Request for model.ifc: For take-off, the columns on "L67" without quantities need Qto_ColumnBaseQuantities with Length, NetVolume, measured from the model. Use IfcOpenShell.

First a look at what the model holds.

```python
import ifcopenshell
import ifcopenshell.util.element
import ifcopenshell.util.unit

model = ifcopenshell.open("model.ifc")
print(model.schema)
for unit_type in ("LENGTHUNIT", "AREAUNIT", "VOLUMEUNIT"):
    print(unit_type, ifcopenshell.util.unit.calculate_unit_scale(model, unit_type))
storey = next(s for s in model.by_type("IfcBuildingStorey") if s.Name == "L67")
columns = [e for e in ifcopenshell.util.element.get_decomposition(storey) if e.is_a("IfcColumn")]
for e in sorted(columns, key=lambda e: e.id()):
    print(e.id(), e.is_a(), e.Name, list(ifcopenshell.util.element.get_psets(e, qtos_only=True)), sep=" | ")
```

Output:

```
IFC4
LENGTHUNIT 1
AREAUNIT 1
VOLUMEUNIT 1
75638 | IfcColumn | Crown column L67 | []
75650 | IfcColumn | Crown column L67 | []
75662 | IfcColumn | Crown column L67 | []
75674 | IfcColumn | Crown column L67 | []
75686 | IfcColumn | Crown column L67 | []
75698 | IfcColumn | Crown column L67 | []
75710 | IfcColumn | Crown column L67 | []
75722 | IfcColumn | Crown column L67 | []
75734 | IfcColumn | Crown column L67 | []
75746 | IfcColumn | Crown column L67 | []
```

```python
import ifcopenshell
import ifcopenshell.api.pset
import ifcopenshell.geom
import ifcopenshell.util.element
import ifcopenshell.util.shape
import ifcopenshell.util.unit

model = ifcopenshell.open("model.ifc")
unit_scale = ifcopenshell.util.unit.calculate_unit_scale(model)
volume_scale = ifcopenshell.util.unit.calculate_unit_scale(model, "VOLUMEUNIT")
settings = ifcopenshell.geom.settings()

storey = next(s for s in model.by_type("IfcBuildingStorey") if s.Name == "L67")
columns = [e for e in ifcopenshell.util.element.get_decomposition(storey) if e.is_a("IfcColumn")]

for e in sorted(columns, key=lambda e: e.id()):
    if ifcopenshell.util.element.get_psets(e, qtos_only=True, should_inherit=False):
        continue
    # Geometry comes back in metres, in the element's own axes.
    shape = ifcopenshell.geom.create_shape(settings, e)
    values = {
        "Length": ifcopenshell.util.shape.get_z(shape.geometry) / unit_scale,
        "NetVolume": ifcopenshell.util.shape.get_volume(shape.geometry) / volume_scale,
    }
    qto = ifcopenshell.api.pset.add_qto(model, product=e, name="Qto_ColumnBaseQuantities")
    ifcopenshell.api.pset.edit_qto(model, qto=qto, properties=values)
    print(e.id(), {k: round(v, 3) for k, v in values.items()})

model.write("model_rev.ifc")
```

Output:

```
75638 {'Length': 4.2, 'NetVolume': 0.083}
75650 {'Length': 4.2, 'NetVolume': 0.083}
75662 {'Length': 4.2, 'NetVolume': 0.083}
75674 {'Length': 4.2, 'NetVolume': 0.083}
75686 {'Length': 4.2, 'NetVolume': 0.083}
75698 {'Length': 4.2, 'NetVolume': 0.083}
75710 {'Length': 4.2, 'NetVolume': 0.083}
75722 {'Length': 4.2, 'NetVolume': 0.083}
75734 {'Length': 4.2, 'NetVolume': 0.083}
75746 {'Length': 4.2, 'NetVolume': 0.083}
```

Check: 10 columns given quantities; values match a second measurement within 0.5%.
